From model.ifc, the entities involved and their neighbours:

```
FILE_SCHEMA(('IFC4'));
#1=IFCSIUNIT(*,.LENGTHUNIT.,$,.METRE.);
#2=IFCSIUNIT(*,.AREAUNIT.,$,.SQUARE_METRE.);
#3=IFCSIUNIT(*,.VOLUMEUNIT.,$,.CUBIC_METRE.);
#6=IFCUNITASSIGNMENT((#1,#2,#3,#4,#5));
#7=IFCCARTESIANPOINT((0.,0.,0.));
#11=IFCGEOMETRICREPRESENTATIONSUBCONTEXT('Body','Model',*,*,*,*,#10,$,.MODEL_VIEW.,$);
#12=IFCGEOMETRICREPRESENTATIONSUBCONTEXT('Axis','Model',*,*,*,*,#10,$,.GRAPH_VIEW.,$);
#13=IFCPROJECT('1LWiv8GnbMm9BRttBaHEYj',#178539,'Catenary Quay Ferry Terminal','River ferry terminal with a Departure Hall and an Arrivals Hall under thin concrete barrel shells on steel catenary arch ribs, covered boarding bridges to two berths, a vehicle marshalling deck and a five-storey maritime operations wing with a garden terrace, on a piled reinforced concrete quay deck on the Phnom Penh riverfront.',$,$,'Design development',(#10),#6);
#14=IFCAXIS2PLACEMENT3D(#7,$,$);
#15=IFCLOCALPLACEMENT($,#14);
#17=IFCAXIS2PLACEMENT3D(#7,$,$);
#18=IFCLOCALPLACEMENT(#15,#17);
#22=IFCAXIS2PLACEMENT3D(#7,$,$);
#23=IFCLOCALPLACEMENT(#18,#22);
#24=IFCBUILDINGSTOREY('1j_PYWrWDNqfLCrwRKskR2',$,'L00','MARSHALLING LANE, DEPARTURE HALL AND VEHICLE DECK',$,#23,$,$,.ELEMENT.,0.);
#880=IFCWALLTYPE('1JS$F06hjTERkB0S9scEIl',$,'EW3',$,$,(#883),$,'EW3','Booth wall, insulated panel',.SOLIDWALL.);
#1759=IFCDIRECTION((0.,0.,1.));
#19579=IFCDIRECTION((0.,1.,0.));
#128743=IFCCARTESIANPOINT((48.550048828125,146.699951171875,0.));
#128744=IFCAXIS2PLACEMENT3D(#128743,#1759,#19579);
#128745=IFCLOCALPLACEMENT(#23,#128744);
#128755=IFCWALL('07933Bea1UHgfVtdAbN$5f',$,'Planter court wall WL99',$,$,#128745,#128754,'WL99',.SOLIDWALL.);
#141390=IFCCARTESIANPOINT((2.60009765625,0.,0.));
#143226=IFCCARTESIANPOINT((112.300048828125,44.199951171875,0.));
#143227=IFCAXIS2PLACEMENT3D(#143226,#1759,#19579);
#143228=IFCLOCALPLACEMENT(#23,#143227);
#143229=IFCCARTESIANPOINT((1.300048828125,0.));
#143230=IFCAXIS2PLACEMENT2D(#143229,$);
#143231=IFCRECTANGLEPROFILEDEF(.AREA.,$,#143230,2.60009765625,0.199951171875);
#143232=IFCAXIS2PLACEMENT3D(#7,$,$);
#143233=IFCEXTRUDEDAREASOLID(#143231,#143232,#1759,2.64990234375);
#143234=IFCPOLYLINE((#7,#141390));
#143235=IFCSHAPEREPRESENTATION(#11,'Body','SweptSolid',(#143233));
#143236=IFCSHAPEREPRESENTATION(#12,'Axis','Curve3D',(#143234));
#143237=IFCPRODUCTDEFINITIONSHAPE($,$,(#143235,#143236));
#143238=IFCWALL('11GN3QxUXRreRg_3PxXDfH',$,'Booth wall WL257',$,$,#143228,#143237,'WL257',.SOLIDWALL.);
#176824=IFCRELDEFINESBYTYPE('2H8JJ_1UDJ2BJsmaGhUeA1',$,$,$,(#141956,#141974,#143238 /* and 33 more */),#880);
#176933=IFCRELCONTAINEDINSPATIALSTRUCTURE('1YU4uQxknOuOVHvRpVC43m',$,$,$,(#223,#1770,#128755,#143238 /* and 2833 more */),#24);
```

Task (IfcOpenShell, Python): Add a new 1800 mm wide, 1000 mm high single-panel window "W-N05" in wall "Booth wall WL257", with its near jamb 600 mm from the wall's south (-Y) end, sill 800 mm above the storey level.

```python
import numpy as np
import ifcopenshell
import ifcopenshell.api.feature
import ifcopenshell.api.geometry
import ifcopenshell.api.root
import ifcopenshell.api.spatial
import ifcopenshell.geom
import ifcopenshell.util.element
import ifcopenshell.util.placement
import ifcopenshell.util.representation
import ifcopenshell.util.shape
import ifcopenshell.util.unit

model = ifcopenshell.open("model.ifc")
unit_scale = ifcopenshell.util.unit.calculate_unit_scale(model)
settings = ifcopenshell.geom.settings()


def volume(element):
    """Net volume in cubic metres, openings subtracted."""
    shape = ifcopenshell.geom.create_shape(settings, element)
    return ifcopenshell.util.shape.get_volume(shape.geometry)


wall = model.by_guid("11GN3QxUXRreRg_3PxXDfH")
storey = ifcopenshell.util.element.get_container(wall, ifc_class="IfcBuildingStorey")
context = ifcopenshell.util.representation.get_context(model, "Model", "Body", "MODEL_VIEW")
before = volume(wall)

width, height, from_end, sill = 1.8, 1, 0.6, 0.8  # metres

# The wall runs along its own X axis, and the end named is its -X end.
wall_shape = ifcopenshell.geom.create_shape(settings, wall)
x, y, z = ifcopenshell.util.shape.get_vertices(wall_shape.geometry).T
start = x.min() + from_end
face, thickness = float(y.min()), float(y.max() - y.min())
wall_matrix = ifcopenshell.util.placement.get_local_placement(wall.ObjectPlacement)
level = ifcopenshell.util.placement.get_local_placement(storey.ObjectPlacement)[2, 3]


def in_wall(x, y):
    """Placement at x, y metres in the wall's axes, at sill height."""
    matrix = wall_matrix.copy()
    matrix[:, 3] = wall_matrix @ np.array([x / unit_scale, y / unit_scale, 0.0, 1.0])
    matrix[2, 3] = level + sill / unit_scale
    return matrix


# Opening: a box that overshoots both wall faces by 50 mm.
opening = ifcopenshell.api.root.create_entity(model, ifc_class="IfcOpeningElement", predefined_type="OPENING")
box = ifcopenshell.api.geometry.add_wall_representation(
    model, context=context, length=width, height=height, thickness=thickness + 0.1
)
ifcopenshell.api.geometry.assign_representation(model, product=opening, representation=box)
ifcopenshell.api.geometry.edit_object_placement(model, product=opening, matrix=in_wall(start, face - 0.05), is_si=False)
ifcopenshell.api.feature.add_feature(model, feature=opening, element=wall)

window = ifcopenshell.api.root.create_entity(model, ifc_class="IfcWindow", name="W-N05", predefined_type="WINDOW")
window.OverallWidth, window.OverallHeight = width / unit_scale, height / unit_scale
window.PartitioningType = "SINGLE_PANEL"
body = ifcopenshell.api.geometry.add_window_representation(
    model,
    context=context,
    overall_width=window.OverallWidth,
    overall_height=window.OverallHeight,
    partition_type="SINGLE_PANEL",
)
ifcopenshell.api.geometry.assign_representation(model, product=window, representation=body)
ifcopenshell.api.spatial.assign_container(model, products=[window], relating_structure=storey)
ifcopenshell.api.feature.add_filling(model, opening=opening, element=window)

# Centre the window in the wall's thickness.
ifcopenshell.api.geometry.edit_object_placement(model, product=window, matrix=in_wall(start, face), is_si=False)
window_shape = ifcopenshell.geom.create_shape(settings, window)
depth = ifcopenshell.util.shape.get_vertices(window_shape.geometry)[:, 1]
offset = face + thickness / 2 - (depth.min() + depth.max()) / 2
ifcopenshell.api.geometry.edit_object_placement(model, product=window, matrix=in_wall(start, offset), is_si=False)

after = volume(wall)

print(f"wall volume {before:.3f} -> {after:.3f} m3")

model.write("model_rev.ifc")
```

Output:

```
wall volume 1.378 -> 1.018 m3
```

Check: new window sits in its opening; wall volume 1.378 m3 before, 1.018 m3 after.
